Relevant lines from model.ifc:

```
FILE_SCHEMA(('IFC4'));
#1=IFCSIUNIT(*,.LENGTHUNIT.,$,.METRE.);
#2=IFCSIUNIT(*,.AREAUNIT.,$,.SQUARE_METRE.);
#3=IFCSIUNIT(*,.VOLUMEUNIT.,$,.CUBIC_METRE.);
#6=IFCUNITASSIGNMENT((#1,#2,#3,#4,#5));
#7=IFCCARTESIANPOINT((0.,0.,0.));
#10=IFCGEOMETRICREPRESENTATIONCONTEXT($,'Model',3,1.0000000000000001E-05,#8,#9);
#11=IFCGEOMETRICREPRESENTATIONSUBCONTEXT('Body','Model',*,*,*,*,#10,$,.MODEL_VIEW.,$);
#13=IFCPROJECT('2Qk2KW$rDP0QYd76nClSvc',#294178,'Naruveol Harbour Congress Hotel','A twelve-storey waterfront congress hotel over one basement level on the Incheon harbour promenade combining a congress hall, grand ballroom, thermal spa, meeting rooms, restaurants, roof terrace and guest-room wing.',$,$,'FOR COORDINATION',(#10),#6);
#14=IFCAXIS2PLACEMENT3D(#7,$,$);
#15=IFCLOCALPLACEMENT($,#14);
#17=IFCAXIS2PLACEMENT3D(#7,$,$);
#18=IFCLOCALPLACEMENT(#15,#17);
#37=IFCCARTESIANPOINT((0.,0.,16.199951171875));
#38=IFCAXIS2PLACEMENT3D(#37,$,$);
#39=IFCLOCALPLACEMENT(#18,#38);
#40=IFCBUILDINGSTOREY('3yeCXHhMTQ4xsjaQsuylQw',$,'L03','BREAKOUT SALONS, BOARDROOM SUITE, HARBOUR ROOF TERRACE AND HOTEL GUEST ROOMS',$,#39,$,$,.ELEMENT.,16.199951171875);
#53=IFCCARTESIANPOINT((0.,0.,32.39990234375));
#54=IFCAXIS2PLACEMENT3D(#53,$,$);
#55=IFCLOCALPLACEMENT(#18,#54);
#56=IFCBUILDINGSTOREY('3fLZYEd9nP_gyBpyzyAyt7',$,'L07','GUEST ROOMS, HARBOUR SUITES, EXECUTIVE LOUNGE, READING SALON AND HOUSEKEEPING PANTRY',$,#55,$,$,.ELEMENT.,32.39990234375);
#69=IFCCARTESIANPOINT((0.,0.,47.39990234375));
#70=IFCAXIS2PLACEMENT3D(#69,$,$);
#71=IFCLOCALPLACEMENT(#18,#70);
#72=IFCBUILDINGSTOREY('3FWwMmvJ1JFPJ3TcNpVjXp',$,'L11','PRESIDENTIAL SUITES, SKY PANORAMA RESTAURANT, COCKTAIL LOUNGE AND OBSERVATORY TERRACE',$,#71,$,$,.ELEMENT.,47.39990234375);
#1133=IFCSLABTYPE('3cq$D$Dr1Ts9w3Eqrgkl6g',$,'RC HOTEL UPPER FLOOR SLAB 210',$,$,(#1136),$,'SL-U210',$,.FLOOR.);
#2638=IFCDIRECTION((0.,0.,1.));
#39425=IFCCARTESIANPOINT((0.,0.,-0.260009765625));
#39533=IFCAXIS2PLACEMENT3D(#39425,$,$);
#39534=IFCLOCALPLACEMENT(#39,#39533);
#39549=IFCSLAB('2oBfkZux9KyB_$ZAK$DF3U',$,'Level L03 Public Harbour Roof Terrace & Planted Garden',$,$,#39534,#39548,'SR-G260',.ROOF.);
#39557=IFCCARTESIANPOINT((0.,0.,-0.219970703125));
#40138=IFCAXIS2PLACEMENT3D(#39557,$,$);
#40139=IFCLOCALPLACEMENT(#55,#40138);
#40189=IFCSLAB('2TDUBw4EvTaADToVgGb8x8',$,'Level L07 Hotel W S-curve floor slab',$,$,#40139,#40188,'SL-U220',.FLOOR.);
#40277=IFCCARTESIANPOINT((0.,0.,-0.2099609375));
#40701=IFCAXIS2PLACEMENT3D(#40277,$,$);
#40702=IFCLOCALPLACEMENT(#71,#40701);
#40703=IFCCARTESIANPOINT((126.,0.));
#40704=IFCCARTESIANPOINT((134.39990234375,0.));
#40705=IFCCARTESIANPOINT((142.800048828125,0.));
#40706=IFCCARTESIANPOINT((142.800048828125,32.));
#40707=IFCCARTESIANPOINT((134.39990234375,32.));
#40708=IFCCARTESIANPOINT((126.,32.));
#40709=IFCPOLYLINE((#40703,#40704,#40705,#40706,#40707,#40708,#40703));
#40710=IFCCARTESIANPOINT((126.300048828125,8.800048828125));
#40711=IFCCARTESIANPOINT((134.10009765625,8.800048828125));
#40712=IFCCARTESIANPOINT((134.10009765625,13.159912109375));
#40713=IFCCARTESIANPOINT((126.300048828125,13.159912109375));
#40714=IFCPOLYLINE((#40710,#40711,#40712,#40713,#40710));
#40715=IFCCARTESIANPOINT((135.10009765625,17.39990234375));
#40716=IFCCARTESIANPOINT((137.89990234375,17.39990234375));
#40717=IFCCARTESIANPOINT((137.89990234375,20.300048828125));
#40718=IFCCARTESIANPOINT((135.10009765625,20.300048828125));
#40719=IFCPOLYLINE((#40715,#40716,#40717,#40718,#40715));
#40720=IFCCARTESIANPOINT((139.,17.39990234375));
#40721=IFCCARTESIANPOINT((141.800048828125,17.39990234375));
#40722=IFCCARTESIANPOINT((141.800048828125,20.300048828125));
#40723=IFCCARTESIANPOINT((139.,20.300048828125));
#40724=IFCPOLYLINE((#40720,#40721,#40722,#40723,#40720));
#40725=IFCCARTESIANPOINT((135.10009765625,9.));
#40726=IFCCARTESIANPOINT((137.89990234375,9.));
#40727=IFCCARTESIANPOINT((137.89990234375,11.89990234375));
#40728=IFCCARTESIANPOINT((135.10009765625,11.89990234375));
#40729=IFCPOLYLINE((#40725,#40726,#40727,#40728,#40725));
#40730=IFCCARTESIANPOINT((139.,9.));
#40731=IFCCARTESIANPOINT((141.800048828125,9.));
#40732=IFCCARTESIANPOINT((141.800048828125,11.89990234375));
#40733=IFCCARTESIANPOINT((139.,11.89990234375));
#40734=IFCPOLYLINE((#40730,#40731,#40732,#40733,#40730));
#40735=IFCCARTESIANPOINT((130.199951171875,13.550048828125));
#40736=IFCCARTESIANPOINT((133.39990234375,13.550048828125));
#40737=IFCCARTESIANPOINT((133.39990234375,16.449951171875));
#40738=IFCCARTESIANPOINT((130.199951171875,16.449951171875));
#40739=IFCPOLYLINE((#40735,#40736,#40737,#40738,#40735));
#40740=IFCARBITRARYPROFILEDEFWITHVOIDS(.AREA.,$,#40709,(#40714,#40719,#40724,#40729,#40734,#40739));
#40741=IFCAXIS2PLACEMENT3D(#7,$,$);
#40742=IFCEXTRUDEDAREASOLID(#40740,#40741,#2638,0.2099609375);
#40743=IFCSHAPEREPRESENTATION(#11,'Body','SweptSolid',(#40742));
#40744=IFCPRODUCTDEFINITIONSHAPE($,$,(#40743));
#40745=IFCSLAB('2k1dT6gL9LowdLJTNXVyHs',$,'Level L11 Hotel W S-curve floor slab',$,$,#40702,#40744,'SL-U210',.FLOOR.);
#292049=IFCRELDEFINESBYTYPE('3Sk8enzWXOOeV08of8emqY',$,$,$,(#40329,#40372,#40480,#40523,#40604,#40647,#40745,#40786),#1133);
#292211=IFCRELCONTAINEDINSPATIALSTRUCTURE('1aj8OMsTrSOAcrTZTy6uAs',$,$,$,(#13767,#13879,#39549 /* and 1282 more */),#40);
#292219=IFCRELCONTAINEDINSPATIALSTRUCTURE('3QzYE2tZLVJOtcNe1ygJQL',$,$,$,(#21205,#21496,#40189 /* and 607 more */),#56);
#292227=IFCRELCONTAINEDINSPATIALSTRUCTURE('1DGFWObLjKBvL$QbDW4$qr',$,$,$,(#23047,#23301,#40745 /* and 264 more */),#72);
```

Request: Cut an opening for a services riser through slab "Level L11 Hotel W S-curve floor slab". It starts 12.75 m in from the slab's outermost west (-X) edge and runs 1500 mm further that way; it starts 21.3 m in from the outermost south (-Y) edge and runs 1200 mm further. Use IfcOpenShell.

```python
import numpy as np
import ifcopenshell
import ifcopenshell.api.feature
import ifcopenshell.api.geometry
import ifcopenshell.api.root
import ifcopenshell.geom
import ifcopenshell.util.placement
import ifcopenshell.util.representation
import ifcopenshell.util.shape
import ifcopenshell.util.unit

model = ifcopenshell.open("model.ifc")
unit_scale = ifcopenshell.util.unit.calculate_unit_scale(model)
settings = ifcopenshell.geom.settings()


def volume(element):
    """Net volume in cubic metres, openings subtracted."""
    shape = ifcopenshell.geom.create_shape(settings, element)
    return ifcopenshell.util.shape.get_volume(shape.geometry)


slab = model.by_guid("2k1dT6gL9LowdLJTNXVyHs")
before = volume(slab)

# Extent in the slab's own axes, in metres. The edges named are its -X and -Y sides.
slab_shape = ifcopenshell.geom.create_shape(settings, slab)
vertices = ifcopenshell.util.shape.get_vertices(slab_shape.geometry)
x_min, y_min, bottom = vertices.min(axis=0)
top = vertices[:, 2].max()

opening = ifcopenshell.api.root.create_entity(model, ifc_class="IfcOpeningElement", name="Services riser opening", predefined_type="OPENING")
context = ifcopenshell.util.representation.get_context(model, "Model", "Body", "MODEL_VIEW")
width, depth = 1.5, 1.2
outline = [(0.0, 0.0), (width, 0.0), (width, depth), (0.0, depth), (0.0, 0.0)]
# Overshoot both faces by 50 mm so the cut is clean.
shape = ifcopenshell.api.geometry.add_slab_representation(
    model, context=context, depth=top - bottom + 0.1, polyline=outline
)
ifcopenshell.api.geometry.assign_representation(model, product=opening, representation=shape)

matrix = ifcopenshell.util.placement.get_local_placement(slab.ObjectPlacement)
matrix[:, 3] = matrix @ np.append(np.array([x_min + 12.75, y_min + 21.3, bottom - 0.05]) / unit_scale, 1.0)
ifcopenshell.api.geometry.edit_object_placement(model, product=opening, matrix=matrix, is_si=False)
ifcopenshell.api.feature.add_feature(model, feature=opening, element=slab)

after = volume(slab)

print(f"slab volume {before:.3f} -> {after:.3f} m3")

model.write("model_updated.ifc")
```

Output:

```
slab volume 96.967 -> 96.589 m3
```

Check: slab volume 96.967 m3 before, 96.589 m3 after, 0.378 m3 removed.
